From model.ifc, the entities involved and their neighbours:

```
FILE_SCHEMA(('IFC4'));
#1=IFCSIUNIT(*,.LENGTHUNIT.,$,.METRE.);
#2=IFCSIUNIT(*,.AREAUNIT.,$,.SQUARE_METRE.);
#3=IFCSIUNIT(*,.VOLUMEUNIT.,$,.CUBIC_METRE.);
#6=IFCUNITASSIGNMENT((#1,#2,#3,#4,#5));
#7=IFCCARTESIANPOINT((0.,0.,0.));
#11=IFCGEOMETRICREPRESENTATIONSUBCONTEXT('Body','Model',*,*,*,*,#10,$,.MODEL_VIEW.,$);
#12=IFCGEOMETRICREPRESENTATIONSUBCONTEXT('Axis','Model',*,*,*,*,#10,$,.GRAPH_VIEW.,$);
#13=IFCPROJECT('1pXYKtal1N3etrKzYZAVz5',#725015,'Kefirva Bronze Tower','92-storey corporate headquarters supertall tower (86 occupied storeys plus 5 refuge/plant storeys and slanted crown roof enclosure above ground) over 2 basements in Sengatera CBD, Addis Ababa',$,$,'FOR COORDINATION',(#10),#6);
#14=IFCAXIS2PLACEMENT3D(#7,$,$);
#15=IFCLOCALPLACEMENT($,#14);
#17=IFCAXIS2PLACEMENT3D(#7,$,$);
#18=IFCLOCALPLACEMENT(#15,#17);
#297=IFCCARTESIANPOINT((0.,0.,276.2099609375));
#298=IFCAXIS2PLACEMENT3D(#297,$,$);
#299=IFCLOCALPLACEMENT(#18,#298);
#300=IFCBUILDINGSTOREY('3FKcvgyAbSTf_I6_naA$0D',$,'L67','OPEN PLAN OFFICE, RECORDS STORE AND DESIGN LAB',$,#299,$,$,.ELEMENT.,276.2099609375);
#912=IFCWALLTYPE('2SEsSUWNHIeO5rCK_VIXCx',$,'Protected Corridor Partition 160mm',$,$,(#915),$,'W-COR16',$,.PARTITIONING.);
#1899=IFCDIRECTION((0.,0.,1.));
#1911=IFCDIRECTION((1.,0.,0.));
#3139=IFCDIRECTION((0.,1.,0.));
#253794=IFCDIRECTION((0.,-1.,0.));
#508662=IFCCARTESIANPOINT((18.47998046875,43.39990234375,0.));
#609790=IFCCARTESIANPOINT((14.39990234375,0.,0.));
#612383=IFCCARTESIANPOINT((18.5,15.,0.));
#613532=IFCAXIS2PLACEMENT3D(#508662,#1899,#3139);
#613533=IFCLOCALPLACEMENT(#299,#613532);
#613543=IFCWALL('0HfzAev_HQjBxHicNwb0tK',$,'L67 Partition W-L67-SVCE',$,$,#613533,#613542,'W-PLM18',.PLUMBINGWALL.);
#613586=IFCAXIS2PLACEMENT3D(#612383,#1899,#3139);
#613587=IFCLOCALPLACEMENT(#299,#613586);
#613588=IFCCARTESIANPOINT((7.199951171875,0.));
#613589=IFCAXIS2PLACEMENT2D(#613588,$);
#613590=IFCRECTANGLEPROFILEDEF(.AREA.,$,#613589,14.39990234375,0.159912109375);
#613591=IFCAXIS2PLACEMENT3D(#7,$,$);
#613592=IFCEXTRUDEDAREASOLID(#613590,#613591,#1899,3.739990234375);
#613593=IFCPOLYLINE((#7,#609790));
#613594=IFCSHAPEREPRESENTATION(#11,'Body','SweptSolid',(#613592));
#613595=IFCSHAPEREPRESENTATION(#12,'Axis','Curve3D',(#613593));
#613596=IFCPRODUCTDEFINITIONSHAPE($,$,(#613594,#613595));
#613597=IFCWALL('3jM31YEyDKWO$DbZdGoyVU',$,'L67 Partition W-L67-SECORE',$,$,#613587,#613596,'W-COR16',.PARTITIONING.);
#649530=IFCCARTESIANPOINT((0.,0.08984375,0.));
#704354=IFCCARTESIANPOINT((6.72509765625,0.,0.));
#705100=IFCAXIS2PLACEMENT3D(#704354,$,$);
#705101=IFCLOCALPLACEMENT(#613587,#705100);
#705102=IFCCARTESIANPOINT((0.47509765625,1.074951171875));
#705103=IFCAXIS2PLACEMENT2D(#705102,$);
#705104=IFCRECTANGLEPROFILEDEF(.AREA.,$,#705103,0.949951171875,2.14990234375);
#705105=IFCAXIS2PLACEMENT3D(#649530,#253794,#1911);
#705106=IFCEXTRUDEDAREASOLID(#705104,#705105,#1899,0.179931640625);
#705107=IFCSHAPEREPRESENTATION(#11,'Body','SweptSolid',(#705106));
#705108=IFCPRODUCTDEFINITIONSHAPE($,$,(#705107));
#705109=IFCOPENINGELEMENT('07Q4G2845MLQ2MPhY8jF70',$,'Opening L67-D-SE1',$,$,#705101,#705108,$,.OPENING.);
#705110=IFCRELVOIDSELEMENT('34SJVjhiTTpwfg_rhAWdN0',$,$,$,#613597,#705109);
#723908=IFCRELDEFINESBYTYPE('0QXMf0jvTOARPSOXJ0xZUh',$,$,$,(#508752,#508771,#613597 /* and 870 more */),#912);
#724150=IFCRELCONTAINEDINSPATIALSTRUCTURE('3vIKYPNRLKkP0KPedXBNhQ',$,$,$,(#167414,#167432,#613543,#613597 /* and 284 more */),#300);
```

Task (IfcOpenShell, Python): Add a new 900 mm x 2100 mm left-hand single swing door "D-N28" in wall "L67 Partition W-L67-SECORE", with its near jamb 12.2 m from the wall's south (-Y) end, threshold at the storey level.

```python
import numpy as np
import ifcopenshell
import ifcopenshell.api.feature
import ifcopenshell.api.geometry
import ifcopenshell.api.root
import ifcopenshell.api.spatial
import ifcopenshell.geom
import ifcopenshell.util.element
import ifcopenshell.util.placement
import ifcopenshell.util.representation
import ifcopenshell.util.shape
import ifcopenshell.util.unit

model = ifcopenshell.open("model.ifc")
unit_scale = ifcopenshell.util.unit.calculate_unit_scale(model)
settings = ifcopenshell.geom.settings()


def volume(element):
    """Net volume in cubic metres, openings subtracted."""
    shape = ifcopenshell.geom.create_shape(settings, element)
    return ifcopenshell.util.shape.get_volume(shape.geometry)


wall = model.by_guid("3jM31YEyDKWO$DbZdGoyVU")
storey = ifcopenshell.util.element.get_container(wall, ifc_class="IfcBuildingStorey")
context = ifcopenshell.util.representation.get_context(model, "Model", "Body", "MODEL_VIEW")
before = volume(wall)

width, height, from_end, sill = 0.9, 2.1, 12.2, 0.0  # metres

# The wall runs along its own X axis, and the end named is its -X end.
wall_shape = ifcopenshell.geom.create_shape(settings, wall)
x, y, z = ifcopenshell.util.shape.get_vertices(wall_shape.geometry).T
start = x.min() + from_end
face, thickness = float(y.min()), float(y.max() - y.min())
wall_matrix = ifcopenshell.util.placement.get_local_placement(wall.ObjectPlacement)
level = ifcopenshell.util.placement.get_local_placement(storey.ObjectPlacement)[2, 3]


def in_wall(x, y):
    """Placement at x, y metres in the wall's axes, at sill height."""
    matrix = wall_matrix.copy()
    matrix[:, 3] = wall_matrix @ np.array([x / unit_scale, y / unit_scale, 0.0, 1.0])
    matrix[2, 3] = level + sill / unit_scale
    return matrix


# Opening: a box that overshoots both wall faces by 50 mm.
opening = ifcopenshell.api.root.create_entity(model, ifc_class="IfcOpeningElement", predefined_type="OPENING")
box = ifcopenshell.api.geometry.add_wall_representation(
    model, context=context, length=width, height=height, thickness=thickness + 0.1
)
ifcopenshell.api.geometry.assign_representation(model, product=opening, representation=box)
ifcopenshell.api.geometry.edit_object_placement(model, product=opening, matrix=in_wall(start, face - 0.05), is_si=False)
ifcopenshell.api.feature.add_feature(model, feature=opening, element=wall)

door = ifcopenshell.api.root.create_entity(model, ifc_class="IfcDoor", name="D-N28", predefined_type="DOOR")
door.OverallWidth, door.OverallHeight = width / unit_scale, height / unit_scale
door.OperationType = "SINGLE_SWING_LEFT"
body = ifcopenshell.api.geometry.add_door_representation(
    model,
    context=context,
    overall_width=door.OverallWidth,
    overall_height=door.OverallHeight,
    operation_type="SINGLE_SWING_LEFT",
    lining_properties={"LiningDepth": thickness / unit_scale, "ThresholdDepth": thickness / unit_scale},
)
ifcopenshell.api.geometry.assign_representation(model, product=door, representation=body)
ifcopenshell.api.spatial.assign_container(model, products=[door], relating_structure=storey)
ifcopenshell.api.feature.add_filling(model, opening=opening, element=door)

# The lining spans the wall, so the door starts at the wall face.
ifcopenshell.api.geometry.edit_object_placement(model, product=door, matrix=in_wall(start, face), is_si=False)

after = volume(wall)

print(f"wall volume {before:.3f} -> {after:.3f} m3")

model.write("model_updated.ifc")
```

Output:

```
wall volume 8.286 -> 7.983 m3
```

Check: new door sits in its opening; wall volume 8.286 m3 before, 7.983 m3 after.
